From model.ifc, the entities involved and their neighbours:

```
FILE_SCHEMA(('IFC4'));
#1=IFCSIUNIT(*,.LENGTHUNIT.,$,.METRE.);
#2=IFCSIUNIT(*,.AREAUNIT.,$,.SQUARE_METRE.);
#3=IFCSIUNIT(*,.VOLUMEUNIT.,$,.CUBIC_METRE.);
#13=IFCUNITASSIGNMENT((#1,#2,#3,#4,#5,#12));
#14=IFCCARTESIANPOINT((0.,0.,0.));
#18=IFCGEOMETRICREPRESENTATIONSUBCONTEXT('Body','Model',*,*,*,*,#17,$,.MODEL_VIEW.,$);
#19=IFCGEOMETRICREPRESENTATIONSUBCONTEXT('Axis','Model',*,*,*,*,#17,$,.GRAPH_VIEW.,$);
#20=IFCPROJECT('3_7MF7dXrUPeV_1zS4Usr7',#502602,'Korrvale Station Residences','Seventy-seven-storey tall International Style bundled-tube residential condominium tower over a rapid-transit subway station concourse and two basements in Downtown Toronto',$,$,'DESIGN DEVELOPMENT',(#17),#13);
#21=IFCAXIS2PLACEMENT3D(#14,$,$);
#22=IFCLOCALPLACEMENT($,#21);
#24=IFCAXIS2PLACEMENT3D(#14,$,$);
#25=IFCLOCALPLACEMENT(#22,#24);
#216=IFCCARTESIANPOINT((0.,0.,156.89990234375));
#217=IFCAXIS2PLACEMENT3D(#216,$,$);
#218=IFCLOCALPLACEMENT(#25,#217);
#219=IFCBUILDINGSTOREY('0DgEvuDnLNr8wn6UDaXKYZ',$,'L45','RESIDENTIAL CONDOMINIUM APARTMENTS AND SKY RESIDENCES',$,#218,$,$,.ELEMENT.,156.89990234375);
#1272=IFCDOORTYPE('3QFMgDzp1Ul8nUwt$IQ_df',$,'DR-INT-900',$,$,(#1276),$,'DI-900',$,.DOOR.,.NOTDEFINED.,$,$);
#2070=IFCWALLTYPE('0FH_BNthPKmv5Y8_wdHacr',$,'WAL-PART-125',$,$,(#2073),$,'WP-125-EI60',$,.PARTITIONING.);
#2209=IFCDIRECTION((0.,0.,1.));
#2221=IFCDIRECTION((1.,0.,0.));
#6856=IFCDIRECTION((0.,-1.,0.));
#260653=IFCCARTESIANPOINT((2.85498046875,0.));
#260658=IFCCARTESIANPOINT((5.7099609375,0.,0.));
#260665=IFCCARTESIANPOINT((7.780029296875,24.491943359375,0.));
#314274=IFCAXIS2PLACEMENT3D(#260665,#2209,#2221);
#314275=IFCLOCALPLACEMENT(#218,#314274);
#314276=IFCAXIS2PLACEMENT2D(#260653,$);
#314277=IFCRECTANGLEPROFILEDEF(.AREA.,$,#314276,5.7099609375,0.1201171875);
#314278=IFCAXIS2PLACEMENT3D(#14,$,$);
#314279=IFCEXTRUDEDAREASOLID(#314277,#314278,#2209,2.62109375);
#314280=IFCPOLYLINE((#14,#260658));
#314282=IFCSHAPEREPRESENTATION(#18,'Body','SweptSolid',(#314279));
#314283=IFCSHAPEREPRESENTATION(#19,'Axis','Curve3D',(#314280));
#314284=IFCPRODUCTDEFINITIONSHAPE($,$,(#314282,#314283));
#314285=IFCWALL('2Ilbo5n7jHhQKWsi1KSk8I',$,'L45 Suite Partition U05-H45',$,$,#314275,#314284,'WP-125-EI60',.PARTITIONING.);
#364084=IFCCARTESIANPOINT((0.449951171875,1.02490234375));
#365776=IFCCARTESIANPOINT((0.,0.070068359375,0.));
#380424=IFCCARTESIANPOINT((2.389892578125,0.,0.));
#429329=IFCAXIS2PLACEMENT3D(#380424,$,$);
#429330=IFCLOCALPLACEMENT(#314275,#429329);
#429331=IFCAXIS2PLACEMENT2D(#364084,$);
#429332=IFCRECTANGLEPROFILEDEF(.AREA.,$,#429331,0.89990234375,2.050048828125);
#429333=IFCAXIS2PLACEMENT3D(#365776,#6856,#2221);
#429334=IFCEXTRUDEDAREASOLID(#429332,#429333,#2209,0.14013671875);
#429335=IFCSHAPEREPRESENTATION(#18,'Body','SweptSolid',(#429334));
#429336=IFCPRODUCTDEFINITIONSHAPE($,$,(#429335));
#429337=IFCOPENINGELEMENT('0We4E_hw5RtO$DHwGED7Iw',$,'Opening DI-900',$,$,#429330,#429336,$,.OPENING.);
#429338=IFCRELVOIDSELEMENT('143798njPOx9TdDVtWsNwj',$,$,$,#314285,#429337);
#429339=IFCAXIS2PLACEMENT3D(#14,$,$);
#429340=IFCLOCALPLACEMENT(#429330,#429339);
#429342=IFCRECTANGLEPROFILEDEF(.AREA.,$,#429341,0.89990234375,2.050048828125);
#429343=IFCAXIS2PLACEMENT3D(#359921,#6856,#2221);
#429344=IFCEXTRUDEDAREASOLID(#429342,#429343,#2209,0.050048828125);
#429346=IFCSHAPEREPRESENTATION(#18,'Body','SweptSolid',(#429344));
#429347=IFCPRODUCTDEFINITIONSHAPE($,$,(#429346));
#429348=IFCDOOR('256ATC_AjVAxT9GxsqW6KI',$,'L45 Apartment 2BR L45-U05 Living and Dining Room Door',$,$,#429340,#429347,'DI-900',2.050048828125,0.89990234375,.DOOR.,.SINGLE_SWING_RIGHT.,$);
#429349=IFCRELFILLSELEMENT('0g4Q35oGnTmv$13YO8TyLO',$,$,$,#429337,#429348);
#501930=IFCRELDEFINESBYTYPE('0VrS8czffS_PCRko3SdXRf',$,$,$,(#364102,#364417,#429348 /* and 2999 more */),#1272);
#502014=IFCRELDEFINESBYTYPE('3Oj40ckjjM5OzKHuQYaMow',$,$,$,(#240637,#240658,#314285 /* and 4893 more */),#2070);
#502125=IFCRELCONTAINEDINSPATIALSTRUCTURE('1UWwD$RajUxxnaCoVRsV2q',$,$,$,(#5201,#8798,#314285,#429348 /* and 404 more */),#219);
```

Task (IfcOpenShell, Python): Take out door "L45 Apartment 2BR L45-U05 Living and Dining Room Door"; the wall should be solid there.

```python
import ifcopenshell
import ifcopenshell.api.feature
import ifcopenshell.api.root
import ifcopenshell.geom
import ifcopenshell.util.shape

model = ifcopenshell.open("model.ifc")
settings = ifcopenshell.geom.settings()


def volume(element):
    """Net volume in cubic metres, openings subtracted."""
    shape = ifcopenshell.geom.create_shape(settings, element)
    return ifcopenshell.util.shape.get_volume(shape.geometry)


door = model.by_guid("256ATC_AjVAxT9GxsqW6KI")
opening = door.FillsVoids[0].RelatingOpeningElement
wall = opening.VoidsElements[0].RelatingBuildingElement
before = volume(wall)

ifcopenshell.api.root.remove_product(model, product=door)
ifcopenshell.api.feature.remove_feature(model, feature=opening)

after = volume(wall)

print(f"wall volume {before:.3f} -> {after:.3f} m3")

model.write("model_rev.ifc")
```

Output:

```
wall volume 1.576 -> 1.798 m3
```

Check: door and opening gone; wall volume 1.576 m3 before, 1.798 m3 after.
